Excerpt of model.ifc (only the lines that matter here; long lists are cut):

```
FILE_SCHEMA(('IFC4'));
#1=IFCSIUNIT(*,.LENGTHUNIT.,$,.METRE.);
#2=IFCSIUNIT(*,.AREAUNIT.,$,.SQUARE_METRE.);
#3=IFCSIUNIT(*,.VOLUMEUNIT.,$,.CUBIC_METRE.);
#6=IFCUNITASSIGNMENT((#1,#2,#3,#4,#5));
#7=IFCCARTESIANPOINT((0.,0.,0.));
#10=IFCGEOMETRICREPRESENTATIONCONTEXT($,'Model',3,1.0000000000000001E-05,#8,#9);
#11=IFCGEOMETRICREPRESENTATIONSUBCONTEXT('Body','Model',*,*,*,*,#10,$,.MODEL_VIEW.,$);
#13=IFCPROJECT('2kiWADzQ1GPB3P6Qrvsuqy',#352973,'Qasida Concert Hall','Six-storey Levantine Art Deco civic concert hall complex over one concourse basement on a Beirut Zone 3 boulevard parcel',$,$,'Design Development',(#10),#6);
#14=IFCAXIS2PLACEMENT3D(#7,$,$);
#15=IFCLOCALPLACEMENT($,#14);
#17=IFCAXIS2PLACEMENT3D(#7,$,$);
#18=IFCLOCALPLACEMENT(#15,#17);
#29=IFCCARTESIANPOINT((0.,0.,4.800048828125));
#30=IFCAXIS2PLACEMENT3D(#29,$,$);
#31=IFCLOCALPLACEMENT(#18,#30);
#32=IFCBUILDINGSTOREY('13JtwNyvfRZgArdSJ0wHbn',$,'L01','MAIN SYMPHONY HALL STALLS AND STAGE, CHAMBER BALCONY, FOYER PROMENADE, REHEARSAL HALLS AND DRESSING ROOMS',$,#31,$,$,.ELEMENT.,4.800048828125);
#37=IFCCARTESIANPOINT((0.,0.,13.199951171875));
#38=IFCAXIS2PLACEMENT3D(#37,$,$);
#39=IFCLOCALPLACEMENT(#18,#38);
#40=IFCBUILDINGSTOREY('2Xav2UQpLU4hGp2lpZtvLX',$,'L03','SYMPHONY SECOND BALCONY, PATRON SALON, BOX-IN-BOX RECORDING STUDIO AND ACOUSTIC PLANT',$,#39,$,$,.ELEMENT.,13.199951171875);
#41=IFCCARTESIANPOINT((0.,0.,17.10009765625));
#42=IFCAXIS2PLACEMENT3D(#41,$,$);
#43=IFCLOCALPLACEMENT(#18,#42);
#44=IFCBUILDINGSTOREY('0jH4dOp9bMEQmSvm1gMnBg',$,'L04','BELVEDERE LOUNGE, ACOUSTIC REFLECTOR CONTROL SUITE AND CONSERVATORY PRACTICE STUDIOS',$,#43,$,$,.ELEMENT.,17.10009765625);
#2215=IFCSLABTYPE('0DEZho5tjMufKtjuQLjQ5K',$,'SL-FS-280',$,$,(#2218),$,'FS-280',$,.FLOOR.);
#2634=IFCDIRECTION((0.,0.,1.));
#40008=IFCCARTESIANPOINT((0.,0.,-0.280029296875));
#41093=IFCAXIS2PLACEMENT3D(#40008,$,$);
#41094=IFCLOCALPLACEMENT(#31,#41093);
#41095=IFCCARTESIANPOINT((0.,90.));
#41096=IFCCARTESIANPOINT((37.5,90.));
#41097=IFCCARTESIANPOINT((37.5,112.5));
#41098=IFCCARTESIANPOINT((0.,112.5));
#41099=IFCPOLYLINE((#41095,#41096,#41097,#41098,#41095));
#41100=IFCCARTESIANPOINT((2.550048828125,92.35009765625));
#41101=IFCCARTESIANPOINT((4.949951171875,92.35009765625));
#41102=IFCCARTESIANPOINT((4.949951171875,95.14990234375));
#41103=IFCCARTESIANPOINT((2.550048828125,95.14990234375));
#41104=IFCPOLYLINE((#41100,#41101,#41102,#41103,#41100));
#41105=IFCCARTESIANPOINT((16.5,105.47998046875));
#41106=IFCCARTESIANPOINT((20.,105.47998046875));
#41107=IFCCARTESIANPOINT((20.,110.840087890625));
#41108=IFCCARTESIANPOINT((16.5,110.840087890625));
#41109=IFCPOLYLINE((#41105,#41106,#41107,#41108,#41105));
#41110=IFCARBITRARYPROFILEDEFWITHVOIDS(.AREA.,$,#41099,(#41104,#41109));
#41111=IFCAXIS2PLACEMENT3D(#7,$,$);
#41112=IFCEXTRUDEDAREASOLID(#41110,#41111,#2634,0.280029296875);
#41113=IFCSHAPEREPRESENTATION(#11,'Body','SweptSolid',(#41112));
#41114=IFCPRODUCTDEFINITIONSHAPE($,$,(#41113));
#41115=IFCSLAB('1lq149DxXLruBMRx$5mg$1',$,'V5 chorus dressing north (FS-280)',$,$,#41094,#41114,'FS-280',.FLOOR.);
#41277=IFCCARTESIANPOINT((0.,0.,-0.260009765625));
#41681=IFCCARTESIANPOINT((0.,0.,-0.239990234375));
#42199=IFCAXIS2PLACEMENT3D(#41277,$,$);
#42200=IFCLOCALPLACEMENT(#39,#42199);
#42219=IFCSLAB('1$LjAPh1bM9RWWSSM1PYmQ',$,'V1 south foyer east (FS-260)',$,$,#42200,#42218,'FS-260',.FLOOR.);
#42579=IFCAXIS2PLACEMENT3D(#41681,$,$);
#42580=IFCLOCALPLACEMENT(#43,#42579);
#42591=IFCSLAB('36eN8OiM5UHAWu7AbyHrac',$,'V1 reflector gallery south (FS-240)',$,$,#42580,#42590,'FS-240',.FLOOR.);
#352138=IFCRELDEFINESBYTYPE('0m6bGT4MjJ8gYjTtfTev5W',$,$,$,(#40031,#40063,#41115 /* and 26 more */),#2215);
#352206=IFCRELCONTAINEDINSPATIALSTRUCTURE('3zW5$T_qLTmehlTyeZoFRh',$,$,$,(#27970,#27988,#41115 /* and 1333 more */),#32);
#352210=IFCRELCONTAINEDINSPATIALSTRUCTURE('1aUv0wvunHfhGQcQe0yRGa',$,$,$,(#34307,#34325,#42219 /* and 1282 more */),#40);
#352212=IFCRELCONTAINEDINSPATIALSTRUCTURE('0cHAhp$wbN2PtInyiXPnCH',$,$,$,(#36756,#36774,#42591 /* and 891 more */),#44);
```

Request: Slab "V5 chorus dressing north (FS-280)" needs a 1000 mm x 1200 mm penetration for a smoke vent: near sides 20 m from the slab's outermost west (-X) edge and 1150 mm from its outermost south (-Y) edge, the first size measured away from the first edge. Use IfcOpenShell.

```python
import numpy as np
import ifcopenshell
import ifcopenshell.api.feature
import ifcopenshell.api.geometry
import ifcopenshell.api.root
import ifcopenshell.geom
import ifcopenshell.util.placement
import ifcopenshell.util.representation
import ifcopenshell.util.shape
import ifcopenshell.util.unit

model = ifcopenshell.open("model.ifc")
unit_scale = ifcopenshell.util.unit.calculate_unit_scale(model)
settings = ifcopenshell.geom.settings()


def volume(element):
    """Net volume in cubic metres, openings subtracted."""
    shape = ifcopenshell.geom.create_shape(settings, element)
    return ifcopenshell.util.shape.get_volume(shape.geometry)


slab = model.by_id(41115)
before = volume(slab)

# Extent in the slab's own axes, in metres. The edges named are its -X and -Y sides.
slab_shape = ifcopenshell.geom.create_shape(settings, slab)
vertices = ifcopenshell.util.shape.get_vertices(slab_shape.geometry)
x_min, y_min, bottom = vertices.min(axis=0)
top = vertices[:, 2].max()

opening = ifcopenshell.api.root.create_entity(model, ifc_class="IfcOpeningElement", name="Smoke vent opening", predefined_type="OPENING")
context = ifcopenshell.util.representation.get_context(model, "Model", "Body", "MODEL_VIEW")
width, depth = 1, 1.2
outline = [(0.0, 0.0), (width, 0.0), (width, depth), (0.0, depth), (0.0, 0.0)]
# Overshoot both faces by 50 mm so the cut is clean.
shape = ifcopenshell.api.geometry.add_slab_representation(
    model, context=context, depth=top - bottom + 0.1, polyline=outline
)
ifcopenshell.api.geometry.assign_representation(model, product=opening, representation=shape)

matrix = ifcopenshell.util.placement.get_local_placement(slab.ObjectPlacement)
matrix[:, 3] = matrix @ np.append(np.array([x_min + 20, y_min + 1.15, bottom - 0.05]) / unit_scale, 1.0)
ifcopenshell.api.geometry.edit_object_placement(model, product=opening, matrix=matrix, is_si=False)
ifcopenshell.api.feature.add_feature(model, feature=opening, element=slab)

after = volume(slab)

print(f"slab volume {before:.3f} -> {after:.3f} m3")

model.write("model_updated.ifc")
```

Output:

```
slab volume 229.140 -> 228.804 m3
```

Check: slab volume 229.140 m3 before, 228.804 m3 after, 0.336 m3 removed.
